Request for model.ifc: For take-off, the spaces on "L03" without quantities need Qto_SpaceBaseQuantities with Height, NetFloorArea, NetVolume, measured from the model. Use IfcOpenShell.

First a look at what the model holds.

```python
import ifcopenshell
import ifcopenshell.util.element
import ifcopenshell.util.unit

model = ifcopenshell.open("model.ifc")
print(model.schema)
for unit_type in ("LENGTHUNIT", "AREAUNIT", "VOLUMEUNIT"):
    print(unit_type, ifcopenshell.util.unit.calculate_unit_scale(model, unit_type))
storey = next(s for s in model.by_type("IfcBuildingStorey") if s.Name == "L03")
spaces = [e for e in ifcopenshell.util.element.get_decomposition(storey) if e.is_a("IfcSpace")]
for e in sorted(spaces, key=lambda e: e.id()):
    print(e.id(), e.is_a(), e.Name, list(ifcopenshell.util.element.get_psets(e, qtos_only=True)), sep=" | ")
```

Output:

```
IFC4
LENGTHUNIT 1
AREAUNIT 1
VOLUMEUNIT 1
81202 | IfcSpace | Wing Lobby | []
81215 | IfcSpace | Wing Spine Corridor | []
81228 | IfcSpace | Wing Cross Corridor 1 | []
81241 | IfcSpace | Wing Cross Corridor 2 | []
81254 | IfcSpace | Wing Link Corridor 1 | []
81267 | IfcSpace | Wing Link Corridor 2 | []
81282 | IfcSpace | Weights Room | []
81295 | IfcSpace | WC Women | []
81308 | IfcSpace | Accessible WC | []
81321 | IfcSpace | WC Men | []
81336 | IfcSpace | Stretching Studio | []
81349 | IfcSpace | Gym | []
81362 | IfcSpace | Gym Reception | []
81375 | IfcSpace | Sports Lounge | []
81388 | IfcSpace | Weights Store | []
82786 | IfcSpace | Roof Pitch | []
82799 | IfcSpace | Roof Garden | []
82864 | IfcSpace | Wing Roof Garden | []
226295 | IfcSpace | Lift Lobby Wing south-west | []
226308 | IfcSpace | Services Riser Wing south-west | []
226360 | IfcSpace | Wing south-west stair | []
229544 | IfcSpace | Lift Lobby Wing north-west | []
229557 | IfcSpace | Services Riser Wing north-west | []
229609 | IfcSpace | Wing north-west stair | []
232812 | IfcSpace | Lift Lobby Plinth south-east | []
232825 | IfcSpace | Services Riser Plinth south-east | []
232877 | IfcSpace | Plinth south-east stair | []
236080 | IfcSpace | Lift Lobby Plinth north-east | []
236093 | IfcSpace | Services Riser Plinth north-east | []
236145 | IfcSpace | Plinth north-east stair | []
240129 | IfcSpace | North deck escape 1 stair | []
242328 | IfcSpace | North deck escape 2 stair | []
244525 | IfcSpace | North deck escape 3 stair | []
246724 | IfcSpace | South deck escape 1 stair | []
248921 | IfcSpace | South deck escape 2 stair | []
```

```python
import ifcopenshell
import ifcopenshell.api.pset
import ifcopenshell.geom
import ifcopenshell.util.element
import ifcopenshell.util.shape
import ifcopenshell.util.unit

model = ifcopenshell.open("model.ifc")
unit_scale = ifcopenshell.util.unit.calculate_unit_scale(model)
area_scale = ifcopenshell.util.unit.calculate_unit_scale(model, "AREAUNIT")
volume_scale = ifcopenshell.util.unit.calculate_unit_scale(model, "VOLUMEUNIT")
settings = ifcopenshell.geom.settings()

storey = next(s for s in model.by_type("IfcBuildingStorey") if s.Name == "L03")
spaces = [e for e in ifcopenshell.util.element.get_decomposition(storey) if e.is_a("IfcSpace")]

for e in sorted(spaces, key=lambda e: e.id()):
    if ifcopenshell.util.element.get_psets(e, qtos_only=True, should_inherit=False):
        continue
    # Geometry comes back in metres, in the element's own axes.
    shape = ifcopenshell.geom.create_shape(settings, e)
    values = {
        "Height": ifcopenshell.util.shape.get_z(shape.geometry) / unit_scale,
        "NetFloorArea": ifcopenshell.util.shape.get_footprint_area(shape.geometry) / area_scale,
        "NetVolume": ifcopenshell.util.shape.get_volume(shape.geometry) / volume_scale,
    }
    qto = ifcopenshell.api.pset.add_qto(model, product=e, name="Qto_SpaceBaseQuantities")
    ifcopenshell.api.pset.edit_qto(model, qto=qto, properties=values)
    print(e.id(), {k: round(v, 3) for k, v in values.items()})

model.write("model-out.ifc")
```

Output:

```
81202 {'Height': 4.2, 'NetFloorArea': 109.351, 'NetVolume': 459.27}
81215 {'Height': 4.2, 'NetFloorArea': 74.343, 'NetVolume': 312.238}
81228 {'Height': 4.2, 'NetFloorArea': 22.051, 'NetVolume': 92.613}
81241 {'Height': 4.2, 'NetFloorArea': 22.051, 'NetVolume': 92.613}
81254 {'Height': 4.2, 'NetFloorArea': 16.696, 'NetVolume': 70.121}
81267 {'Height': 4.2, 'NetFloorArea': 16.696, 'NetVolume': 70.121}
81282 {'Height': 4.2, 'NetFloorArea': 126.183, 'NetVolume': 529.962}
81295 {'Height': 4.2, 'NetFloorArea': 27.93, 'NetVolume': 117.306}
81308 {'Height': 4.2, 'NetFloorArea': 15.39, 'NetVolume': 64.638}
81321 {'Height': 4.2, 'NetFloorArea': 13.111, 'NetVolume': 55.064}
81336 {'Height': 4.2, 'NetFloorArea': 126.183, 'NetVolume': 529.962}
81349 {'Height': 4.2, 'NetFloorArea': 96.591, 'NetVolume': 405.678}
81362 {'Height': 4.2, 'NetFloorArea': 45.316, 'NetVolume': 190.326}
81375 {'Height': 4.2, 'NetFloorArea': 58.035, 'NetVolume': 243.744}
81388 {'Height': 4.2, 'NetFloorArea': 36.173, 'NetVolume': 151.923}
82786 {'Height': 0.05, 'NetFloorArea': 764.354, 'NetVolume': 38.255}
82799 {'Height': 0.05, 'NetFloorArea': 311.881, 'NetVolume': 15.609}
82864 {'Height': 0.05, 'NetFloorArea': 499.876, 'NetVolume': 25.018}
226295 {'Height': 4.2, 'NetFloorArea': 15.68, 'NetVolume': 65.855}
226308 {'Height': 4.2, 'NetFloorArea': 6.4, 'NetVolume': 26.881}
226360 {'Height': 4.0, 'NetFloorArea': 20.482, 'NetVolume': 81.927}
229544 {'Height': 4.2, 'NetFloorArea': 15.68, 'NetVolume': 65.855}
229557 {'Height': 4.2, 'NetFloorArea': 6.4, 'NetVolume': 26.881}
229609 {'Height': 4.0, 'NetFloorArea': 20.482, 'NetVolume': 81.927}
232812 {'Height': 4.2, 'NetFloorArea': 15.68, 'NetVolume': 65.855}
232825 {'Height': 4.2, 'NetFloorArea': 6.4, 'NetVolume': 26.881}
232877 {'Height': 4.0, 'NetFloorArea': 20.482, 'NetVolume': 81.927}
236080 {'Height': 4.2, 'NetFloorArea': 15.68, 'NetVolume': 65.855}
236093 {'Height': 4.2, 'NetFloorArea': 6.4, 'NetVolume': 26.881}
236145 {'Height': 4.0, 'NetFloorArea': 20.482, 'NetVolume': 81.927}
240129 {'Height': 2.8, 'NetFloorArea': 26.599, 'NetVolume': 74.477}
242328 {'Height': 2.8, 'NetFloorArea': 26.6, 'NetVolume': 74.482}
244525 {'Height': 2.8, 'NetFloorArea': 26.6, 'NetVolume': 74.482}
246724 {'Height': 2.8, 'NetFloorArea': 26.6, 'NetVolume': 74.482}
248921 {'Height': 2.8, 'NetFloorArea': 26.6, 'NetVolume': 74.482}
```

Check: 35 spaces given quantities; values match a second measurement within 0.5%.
